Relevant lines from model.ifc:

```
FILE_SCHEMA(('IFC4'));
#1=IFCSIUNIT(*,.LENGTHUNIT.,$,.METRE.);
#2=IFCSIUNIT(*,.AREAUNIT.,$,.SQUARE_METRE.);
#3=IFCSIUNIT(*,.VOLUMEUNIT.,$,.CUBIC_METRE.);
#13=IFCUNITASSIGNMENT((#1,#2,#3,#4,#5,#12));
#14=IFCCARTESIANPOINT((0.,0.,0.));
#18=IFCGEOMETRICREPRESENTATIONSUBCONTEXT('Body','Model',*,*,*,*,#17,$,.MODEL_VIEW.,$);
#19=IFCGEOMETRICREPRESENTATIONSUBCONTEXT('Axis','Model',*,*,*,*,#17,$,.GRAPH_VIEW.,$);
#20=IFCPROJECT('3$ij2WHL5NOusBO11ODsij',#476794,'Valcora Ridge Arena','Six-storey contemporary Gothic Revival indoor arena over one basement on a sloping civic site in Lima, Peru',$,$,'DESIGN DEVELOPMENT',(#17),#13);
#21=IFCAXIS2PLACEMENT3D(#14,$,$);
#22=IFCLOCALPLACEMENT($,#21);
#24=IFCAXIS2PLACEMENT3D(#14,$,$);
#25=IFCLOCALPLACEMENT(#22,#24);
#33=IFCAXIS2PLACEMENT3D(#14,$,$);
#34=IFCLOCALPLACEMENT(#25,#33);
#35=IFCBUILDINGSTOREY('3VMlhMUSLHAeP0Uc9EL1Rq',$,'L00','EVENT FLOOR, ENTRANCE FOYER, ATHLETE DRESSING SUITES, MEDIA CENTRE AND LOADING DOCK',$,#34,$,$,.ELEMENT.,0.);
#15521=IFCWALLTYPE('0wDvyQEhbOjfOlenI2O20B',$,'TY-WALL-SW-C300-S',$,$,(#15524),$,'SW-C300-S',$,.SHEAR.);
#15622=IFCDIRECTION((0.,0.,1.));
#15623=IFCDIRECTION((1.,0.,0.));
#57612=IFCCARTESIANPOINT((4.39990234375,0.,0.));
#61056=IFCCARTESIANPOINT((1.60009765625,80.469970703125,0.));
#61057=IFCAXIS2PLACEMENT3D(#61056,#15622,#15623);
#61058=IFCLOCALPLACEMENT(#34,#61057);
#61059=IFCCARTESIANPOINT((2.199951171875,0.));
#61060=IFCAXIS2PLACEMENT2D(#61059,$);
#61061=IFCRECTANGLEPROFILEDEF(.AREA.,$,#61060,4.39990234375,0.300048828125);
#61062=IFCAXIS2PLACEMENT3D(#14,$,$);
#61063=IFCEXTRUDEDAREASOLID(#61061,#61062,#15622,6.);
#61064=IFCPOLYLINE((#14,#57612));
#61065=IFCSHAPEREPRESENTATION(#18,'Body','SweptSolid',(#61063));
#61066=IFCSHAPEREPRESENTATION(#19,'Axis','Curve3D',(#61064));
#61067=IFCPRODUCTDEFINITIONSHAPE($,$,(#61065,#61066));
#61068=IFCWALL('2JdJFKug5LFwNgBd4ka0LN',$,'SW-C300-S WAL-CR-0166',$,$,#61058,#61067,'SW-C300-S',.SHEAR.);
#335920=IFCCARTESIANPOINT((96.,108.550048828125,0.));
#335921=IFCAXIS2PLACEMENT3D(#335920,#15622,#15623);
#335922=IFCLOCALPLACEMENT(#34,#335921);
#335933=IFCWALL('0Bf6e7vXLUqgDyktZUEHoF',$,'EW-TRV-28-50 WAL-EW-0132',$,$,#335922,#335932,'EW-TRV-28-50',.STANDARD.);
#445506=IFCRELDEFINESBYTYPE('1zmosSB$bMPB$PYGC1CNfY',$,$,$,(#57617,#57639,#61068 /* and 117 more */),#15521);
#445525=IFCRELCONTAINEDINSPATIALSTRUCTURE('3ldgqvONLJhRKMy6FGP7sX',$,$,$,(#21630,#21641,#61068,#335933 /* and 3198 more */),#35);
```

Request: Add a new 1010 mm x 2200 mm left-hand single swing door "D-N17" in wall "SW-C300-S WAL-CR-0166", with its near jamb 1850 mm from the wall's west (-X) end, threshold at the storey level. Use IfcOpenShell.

```python
import numpy as np
import ifcopenshell
import ifcopenshell.api.feature
import ifcopenshell.api.geometry
import ifcopenshell.api.root
import ifcopenshell.api.spatial
import ifcopenshell.geom
import ifcopenshell.util.element
import ifcopenshell.util.placement
import ifcopenshell.util.representation
import ifcopenshell.util.shape
import ifcopenshell.util.unit

model = ifcopenshell.open("model.ifc")
unit_scale = ifcopenshell.util.unit.calculate_unit_scale(model)
settings = ifcopenshell.geom.settings()


def volume(element):
    """Net volume in cubic metres, openings subtracted."""
    shape = ifcopenshell.geom.create_shape(settings, element)
    return ifcopenshell.util.shape.get_volume(shape.geometry)


wall = model.by_id(61068)
storey = ifcopenshell.util.element.get_container(wall, ifc_class="IfcBuildingStorey")
context = ifcopenshell.util.representation.get_context(model, "Model", "Body", "MODEL_VIEW")
before = volume(wall)

width, height, from_end, sill = 1.01, 2.2, 1.85, 0.0  # metres

# The wall runs along its own X axis, and the end named is its -X end.
wall_shape = ifcopenshell.geom.create_shape(settings, wall)
x, y, z = ifcopenshell.util.shape.get_vertices(wall_shape.geometry).T
start = x.min() + from_end
face, thickness = float(y.min()), float(y.max() - y.min())
wall_matrix = ifcopenshell.util.placement.get_local_placement(wall.ObjectPlacement)
level = ifcopenshell.util.placement.get_local_placement(storey.ObjectPlacement)[2, 3]


def in_wall(x, y):
    """Placement at x, y metres in the wall's axes, at sill height."""
    matrix = wall_matrix.copy()
    matrix[:, 3] = wall_matrix @ np.array([x / unit_scale, y / unit_scale, 0.0, 1.0])
    matrix[2, 3] = level + sill / unit_scale
    return matrix


# Opening: a box that overshoots both wall faces by 50 mm.
opening = ifcopenshell.api.root.create_entity(model, ifc_class="IfcOpeningElement", predefined_type="OPENING")
box = ifcopenshell.api.geometry.add_wall_representation(
    model, context=context, length=width, height=height, thickness=thickness + 0.1
)
ifcopenshell.api.geometry.assign_representation(model, product=opening, representation=box)
ifcopenshell.api.geometry.edit_object_placement(model, product=opening, matrix=in_wall(start, face - 0.05), is_si=False)
ifcopenshell.api.feature.add_feature(model, feature=opening, element=wall)

door = ifcopenshell.api.root.create_entity(model, ifc_class="IfcDoor", name="D-N17", predefined_type="DOOR")
door.OverallWidth, door.OverallHeight = width / unit_scale, height / unit_scale
door.OperationType = "SINGLE_SWING_LEFT"
body = ifcopenshell.api.geometry.add_door_representation(
    model,
    context=context,
    overall_width=door.OverallWidth,
    overall_height=door.OverallHeight,
    operation_type="SINGLE_SWING_LEFT",
    lining_properties={"LiningDepth": thickness / unit_scale, "ThresholdDepth": thickness / unit_scale},
)
ifcopenshell.api.geometry.assign_representation(model, product=door, representation=body)
ifcopenshell.api.spatial.assign_container(model, products=[door], relating_structure=storey)
ifcopenshell.api.feature.add_filling(model, opening=opening, element=door)

# The lining spans the wall, so the door starts at the wall face.
ifcopenshell.api.geometry.edit_object_placement(model, product=door, matrix=in_wall(start, face), is_si=False)

after = volume(wall)

print(f"wall volume {before:.3f} -> {after:.3f} m3")

model.write("model_rev.ifc")
```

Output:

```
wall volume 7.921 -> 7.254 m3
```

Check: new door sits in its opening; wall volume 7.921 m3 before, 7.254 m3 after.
